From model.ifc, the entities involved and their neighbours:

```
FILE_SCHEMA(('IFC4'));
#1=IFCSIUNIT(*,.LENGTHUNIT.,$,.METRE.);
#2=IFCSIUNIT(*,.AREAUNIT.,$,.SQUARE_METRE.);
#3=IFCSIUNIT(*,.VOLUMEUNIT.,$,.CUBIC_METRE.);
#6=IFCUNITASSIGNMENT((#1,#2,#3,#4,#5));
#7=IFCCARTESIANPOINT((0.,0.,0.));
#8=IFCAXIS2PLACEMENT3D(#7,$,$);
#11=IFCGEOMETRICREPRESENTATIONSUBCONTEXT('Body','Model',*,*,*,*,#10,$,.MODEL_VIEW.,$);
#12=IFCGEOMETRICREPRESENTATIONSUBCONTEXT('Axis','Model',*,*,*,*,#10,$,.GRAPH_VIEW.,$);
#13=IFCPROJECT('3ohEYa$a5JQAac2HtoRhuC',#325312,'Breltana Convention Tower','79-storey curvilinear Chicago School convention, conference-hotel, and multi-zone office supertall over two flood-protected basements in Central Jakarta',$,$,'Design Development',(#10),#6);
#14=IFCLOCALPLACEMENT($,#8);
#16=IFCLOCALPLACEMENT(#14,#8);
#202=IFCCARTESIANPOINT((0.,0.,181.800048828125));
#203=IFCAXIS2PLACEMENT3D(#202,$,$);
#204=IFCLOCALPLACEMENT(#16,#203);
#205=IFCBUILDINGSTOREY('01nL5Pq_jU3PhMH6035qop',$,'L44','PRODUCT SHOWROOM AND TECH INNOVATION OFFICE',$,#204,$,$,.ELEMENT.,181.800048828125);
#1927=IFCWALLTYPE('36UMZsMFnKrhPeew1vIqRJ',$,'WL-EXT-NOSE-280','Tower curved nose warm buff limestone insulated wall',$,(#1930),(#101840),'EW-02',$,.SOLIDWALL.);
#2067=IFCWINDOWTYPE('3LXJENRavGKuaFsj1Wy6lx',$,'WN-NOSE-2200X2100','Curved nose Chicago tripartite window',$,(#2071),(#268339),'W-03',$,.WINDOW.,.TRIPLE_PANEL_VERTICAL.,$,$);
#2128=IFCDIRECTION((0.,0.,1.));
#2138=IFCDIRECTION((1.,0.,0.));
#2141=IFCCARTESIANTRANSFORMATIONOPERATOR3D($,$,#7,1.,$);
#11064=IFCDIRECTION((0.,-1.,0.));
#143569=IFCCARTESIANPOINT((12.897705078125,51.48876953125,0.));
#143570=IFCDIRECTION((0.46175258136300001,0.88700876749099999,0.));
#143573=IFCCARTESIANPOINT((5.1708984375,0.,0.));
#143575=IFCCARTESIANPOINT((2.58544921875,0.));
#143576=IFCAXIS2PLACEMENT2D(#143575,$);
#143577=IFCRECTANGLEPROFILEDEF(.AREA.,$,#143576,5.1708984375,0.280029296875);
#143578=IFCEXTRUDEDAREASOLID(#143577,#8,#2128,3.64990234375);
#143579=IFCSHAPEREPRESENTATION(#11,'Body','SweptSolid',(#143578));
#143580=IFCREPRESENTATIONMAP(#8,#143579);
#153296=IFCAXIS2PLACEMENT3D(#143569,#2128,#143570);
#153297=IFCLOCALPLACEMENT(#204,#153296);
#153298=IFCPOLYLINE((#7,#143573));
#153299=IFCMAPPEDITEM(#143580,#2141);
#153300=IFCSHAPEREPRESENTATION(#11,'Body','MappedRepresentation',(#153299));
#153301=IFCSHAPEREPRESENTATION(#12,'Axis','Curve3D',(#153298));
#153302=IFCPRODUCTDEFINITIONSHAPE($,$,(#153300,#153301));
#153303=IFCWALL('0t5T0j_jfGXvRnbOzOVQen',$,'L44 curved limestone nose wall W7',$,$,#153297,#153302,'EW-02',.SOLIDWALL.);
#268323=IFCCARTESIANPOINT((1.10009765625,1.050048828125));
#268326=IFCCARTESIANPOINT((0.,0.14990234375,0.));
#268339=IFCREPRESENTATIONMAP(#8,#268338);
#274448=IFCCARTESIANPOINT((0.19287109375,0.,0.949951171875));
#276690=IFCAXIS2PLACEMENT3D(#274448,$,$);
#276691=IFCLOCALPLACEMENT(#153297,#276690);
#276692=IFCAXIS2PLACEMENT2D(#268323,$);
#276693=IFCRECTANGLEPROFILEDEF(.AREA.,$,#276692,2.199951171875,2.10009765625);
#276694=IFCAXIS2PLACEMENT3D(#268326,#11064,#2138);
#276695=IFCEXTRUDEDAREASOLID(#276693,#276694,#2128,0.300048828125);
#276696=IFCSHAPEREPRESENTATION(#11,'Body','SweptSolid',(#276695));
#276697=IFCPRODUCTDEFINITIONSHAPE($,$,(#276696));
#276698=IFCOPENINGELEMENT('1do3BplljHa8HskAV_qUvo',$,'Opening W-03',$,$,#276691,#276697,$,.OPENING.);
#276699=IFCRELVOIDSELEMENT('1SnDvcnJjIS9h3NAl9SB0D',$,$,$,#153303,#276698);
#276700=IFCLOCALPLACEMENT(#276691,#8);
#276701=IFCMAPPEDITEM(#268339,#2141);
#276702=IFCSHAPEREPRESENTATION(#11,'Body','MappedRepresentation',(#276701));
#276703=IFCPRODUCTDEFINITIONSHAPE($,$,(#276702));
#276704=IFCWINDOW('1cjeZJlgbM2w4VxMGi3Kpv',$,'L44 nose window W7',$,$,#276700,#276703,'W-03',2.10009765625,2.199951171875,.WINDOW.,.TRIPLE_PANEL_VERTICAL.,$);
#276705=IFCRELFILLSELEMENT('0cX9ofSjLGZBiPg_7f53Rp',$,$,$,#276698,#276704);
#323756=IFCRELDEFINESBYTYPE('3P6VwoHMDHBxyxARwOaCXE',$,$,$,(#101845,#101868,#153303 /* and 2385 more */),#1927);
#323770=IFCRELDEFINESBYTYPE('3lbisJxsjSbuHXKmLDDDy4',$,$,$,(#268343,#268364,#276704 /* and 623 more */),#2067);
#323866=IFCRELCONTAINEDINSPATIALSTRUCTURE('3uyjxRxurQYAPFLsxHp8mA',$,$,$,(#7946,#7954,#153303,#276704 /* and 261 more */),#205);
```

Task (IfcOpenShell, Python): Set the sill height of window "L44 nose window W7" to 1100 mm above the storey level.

```python
import numpy as np
import ifcopenshell
import ifcopenshell.api.geometry
import ifcopenshell.geom
import ifcopenshell.util.element
import ifcopenshell.util.placement
import ifcopenshell.util.shape
import ifcopenshell.util.unit

model = ifcopenshell.open("model.ifc")
unit_scale = ifcopenshell.util.unit.calculate_unit_scale(model)

window = model.by_id(276704)
opening = window.FillsVoids[0].RelatingOpeningElement
storey = ifcopenshell.util.element.get_container(window, ifc_class="IfcBuildingStorey")
level = ifcopenshell.util.placement.get_local_placement(storey.ObjectPlacement)[2, 3]

# The opening's origin need not be at the sill, so measure its lowest point.
shape = ifcopenshell.geom.create_shape(ifcopenshell.geom.settings(), opening)
bottom = ifcopenshell.util.shape.get_shape_bottom_elevation(shape, shape.geometry) / unit_scale
dz = level + 1.1 - bottom

shift = np.array([0.0, 0.0, dz])
# The window is placed relative to its opening, so it follows when the opening moves.
matrix = ifcopenshell.util.placement.get_local_placement(opening.ObjectPlacement)
matrix[:3, 3] += shift
ifcopenshell.api.geometry.edit_object_placement(
    model, product=opening, matrix=matrix, is_si=False, should_transform_children=True
)

print(f"moved by {dz * unit_scale:+.3f} m")

model.write("model_rev.ifc")
```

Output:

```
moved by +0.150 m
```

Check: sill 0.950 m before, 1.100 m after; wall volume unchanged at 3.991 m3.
